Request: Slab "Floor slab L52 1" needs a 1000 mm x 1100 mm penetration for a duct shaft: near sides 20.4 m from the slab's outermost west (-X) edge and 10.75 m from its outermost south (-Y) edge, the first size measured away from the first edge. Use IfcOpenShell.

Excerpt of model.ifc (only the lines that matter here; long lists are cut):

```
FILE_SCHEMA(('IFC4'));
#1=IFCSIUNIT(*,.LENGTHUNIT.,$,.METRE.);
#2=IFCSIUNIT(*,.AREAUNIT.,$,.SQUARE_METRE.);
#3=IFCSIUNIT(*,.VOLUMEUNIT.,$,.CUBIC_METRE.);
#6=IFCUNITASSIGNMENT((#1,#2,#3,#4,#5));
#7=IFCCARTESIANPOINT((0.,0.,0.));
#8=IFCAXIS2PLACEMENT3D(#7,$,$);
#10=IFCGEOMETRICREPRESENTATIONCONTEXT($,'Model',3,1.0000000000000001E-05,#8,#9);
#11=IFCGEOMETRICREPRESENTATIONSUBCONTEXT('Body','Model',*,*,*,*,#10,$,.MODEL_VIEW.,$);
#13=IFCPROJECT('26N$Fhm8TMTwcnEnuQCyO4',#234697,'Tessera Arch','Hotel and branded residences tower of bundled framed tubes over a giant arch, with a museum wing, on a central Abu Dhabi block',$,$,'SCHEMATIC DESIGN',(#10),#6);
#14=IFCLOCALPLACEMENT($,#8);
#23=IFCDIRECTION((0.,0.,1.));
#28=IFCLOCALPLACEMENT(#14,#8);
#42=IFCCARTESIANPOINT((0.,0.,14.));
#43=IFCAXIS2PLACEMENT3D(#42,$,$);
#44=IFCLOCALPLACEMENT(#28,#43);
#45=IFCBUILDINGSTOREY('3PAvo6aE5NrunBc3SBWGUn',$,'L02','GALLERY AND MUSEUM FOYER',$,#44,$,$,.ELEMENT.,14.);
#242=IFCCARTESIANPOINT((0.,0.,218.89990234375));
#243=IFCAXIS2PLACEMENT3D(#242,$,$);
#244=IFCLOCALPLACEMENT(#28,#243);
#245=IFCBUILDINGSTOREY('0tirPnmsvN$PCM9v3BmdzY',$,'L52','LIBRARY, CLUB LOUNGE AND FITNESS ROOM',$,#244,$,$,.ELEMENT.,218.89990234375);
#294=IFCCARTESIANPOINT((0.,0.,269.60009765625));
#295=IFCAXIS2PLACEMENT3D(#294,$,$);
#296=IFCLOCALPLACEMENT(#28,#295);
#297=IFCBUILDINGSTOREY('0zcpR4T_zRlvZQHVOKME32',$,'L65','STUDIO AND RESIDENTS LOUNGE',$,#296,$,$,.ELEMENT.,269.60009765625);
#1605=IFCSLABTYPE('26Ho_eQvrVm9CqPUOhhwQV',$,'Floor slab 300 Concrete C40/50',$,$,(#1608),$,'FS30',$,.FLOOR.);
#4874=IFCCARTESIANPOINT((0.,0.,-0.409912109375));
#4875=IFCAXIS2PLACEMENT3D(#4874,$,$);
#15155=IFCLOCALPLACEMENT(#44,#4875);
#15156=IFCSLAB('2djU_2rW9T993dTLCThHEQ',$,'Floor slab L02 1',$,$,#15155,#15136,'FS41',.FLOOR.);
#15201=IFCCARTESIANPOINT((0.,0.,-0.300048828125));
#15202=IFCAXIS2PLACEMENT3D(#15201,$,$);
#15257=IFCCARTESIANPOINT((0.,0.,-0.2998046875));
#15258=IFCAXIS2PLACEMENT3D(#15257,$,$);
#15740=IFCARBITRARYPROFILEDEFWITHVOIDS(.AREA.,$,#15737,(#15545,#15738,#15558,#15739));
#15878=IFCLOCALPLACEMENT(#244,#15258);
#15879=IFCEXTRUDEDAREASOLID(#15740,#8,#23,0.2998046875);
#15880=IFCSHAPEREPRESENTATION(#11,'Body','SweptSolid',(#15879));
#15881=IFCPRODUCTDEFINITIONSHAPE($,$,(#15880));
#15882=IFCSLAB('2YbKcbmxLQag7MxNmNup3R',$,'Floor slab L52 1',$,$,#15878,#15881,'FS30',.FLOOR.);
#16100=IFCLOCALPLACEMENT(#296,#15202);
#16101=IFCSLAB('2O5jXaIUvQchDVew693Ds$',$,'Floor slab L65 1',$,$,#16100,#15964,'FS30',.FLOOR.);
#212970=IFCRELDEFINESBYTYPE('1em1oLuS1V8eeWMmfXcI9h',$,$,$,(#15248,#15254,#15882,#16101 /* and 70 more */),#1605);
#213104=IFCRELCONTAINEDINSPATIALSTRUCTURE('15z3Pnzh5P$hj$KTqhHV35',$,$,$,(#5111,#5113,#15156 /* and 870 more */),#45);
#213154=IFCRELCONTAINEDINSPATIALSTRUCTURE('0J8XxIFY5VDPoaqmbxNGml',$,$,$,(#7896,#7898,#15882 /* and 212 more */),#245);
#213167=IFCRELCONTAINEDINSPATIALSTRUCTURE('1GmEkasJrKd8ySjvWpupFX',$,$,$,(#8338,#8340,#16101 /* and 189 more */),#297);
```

```python
import numpy as np
import ifcopenshell
import ifcopenshell.api.feature
import ifcopenshell.api.geometry
import ifcopenshell.api.root
import ifcopenshell.geom
import ifcopenshell.util.placement
import ifcopenshell.util.representation
import ifcopenshell.util.shape
import ifcopenshell.util.unit

model = ifcopenshell.open("model.ifc")
unit_scale = ifcopenshell.util.unit.calculate_unit_scale(model)
settings = ifcopenshell.geom.settings()


def volume(element):
    """Net volume in cubic metres, openings subtracted."""
    shape = ifcopenshell.geom.create_shape(settings, element)
    return ifcopenshell.util.shape.get_volume(shape.geometry)


slab = model.by_id(15882)
before = volume(slab)

# Extent in the slab's own axes, in metres. The edges named are its -X and -Y sides.
slab_shape = ifcopenshell.geom.create_shape(settings, slab)
vertices = ifcopenshell.util.shape.get_vertices(slab_shape.geometry)
x_min, y_min, bottom = vertices.min(axis=0)
top = vertices[:, 2].max()

opening = ifcopenshell.api.root.create_entity(model, ifc_class="IfcOpeningElement", name="Duct shaft opening", predefined_type="OPENING")
context = ifcopenshell.util.representation.get_context(model, "Model", "Body", "MODEL_VIEW")
width, depth = 1, 1.1
outline = [(0.0, 0.0), (width, 0.0), (width, depth), (0.0, depth), (0.0, 0.0)]
# Overshoot both faces by 50 mm so the cut is clean.
shape = ifcopenshell.api.geometry.add_slab_representation(
    model, context=context, depth=top - bottom + 0.1, polyline=outline
)
ifcopenshell.api.geometry.assign_representation(model, product=opening, representation=shape)

matrix = ifcopenshell.util.placement.get_local_placement(slab.ObjectPlacement)
matrix[:, 3] = matrix @ np.append(np.array([x_min + 20.4, y_min + 10.75, bottom - 0.05]) / unit_scale, 1.0)
ifcopenshell.api.geometry.edit_object_placement(model, product=opening, matrix=matrix, is_si=False)
ifcopenshell.api.feature.add_feature(model, feature=opening, element=slab)

after = volume(slab)

print(f"slab volume {before:.3f} -> {after:.3f} m3")

model.write("model-out.ifc")
```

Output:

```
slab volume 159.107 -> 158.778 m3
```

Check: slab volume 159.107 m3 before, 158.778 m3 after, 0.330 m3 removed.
